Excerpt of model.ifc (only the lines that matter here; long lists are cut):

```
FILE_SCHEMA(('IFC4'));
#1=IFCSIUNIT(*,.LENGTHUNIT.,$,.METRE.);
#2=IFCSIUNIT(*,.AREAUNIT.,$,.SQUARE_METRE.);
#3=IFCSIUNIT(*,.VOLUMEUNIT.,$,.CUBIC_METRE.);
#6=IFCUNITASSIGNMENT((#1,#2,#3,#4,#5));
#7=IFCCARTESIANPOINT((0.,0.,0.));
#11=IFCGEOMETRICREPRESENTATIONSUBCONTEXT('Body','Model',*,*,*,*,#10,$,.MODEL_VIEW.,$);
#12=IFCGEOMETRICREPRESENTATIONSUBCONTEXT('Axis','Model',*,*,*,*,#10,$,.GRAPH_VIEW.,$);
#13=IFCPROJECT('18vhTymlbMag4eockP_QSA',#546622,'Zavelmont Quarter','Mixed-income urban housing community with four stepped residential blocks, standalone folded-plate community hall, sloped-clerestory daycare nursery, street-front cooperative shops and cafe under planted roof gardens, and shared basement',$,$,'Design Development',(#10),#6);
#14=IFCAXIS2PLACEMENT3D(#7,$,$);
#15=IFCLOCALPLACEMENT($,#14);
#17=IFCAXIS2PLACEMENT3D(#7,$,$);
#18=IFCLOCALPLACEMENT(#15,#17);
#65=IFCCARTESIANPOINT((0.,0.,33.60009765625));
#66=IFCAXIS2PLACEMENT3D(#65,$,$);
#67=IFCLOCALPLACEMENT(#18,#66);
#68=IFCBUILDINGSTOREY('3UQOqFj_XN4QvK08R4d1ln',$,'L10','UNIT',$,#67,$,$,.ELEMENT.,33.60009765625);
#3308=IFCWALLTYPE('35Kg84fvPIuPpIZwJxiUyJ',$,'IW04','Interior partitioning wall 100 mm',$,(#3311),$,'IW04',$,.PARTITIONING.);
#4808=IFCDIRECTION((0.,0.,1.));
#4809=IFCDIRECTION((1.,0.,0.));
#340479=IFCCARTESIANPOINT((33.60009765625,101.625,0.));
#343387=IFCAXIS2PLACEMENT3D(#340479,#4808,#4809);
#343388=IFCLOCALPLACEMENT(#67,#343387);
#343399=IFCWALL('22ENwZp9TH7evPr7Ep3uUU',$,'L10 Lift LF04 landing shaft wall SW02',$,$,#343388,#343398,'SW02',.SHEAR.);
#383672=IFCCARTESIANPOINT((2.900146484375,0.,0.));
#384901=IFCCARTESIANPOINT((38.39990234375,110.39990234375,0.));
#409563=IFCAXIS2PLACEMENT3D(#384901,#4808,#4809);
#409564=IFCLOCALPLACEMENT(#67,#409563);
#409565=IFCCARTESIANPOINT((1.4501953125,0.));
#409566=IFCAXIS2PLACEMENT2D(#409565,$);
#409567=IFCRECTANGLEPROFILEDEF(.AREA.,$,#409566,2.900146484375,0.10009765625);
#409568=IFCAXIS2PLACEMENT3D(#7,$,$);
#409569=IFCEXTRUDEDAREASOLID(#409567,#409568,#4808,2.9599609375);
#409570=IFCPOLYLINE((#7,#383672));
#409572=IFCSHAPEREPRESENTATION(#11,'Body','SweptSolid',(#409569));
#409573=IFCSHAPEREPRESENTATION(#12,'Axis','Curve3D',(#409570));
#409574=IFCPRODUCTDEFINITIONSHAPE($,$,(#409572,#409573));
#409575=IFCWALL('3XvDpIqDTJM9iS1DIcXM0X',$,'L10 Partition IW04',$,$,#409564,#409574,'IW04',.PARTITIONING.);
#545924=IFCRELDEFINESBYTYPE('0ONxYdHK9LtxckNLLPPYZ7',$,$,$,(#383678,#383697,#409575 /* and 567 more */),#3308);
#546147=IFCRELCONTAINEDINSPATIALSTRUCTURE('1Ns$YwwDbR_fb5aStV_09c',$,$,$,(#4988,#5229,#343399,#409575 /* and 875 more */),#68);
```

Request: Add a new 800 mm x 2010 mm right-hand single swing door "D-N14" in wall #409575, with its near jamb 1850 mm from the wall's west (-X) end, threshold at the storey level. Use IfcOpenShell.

```python
import numpy as np
import ifcopenshell
import ifcopenshell.api.feature
import ifcopenshell.api.geometry
import ifcopenshell.api.root
import ifcopenshell.api.spatial
import ifcopenshell.geom
import ifcopenshell.util.element
import ifcopenshell.util.placement
import ifcopenshell.util.representation
import ifcopenshell.util.shape
import ifcopenshell.util.unit

model = ifcopenshell.open("model.ifc")
unit_scale = ifcopenshell.util.unit.calculate_unit_scale(model)
settings = ifcopenshell.geom.settings()


def volume(element):
    """Net volume in cubic metres, openings subtracted."""
    shape = ifcopenshell.geom.create_shape(settings, element)
    return ifcopenshell.util.shape.get_volume(shape.geometry)


wall = model.by_id(409575)
storey = ifcopenshell.util.element.get_container(wall, ifc_class="IfcBuildingStorey")
context = ifcopenshell.util.representation.get_context(model, "Model", "Body", "MODEL_VIEW")
before = volume(wall)

width, height, from_end, sill = 0.8, 2.01, 1.85, 0.0  # metres

# The wall runs along its own X axis, and the end named is its -X end.
wall_shape = ifcopenshell.geom.create_shape(settings, wall)
x, y, z = ifcopenshell.util.shape.get_vertices(wall_shape.geometry).T
start = x.min() + from_end
face, thickness = float(y.min()), float(y.max() - y.min())
wall_matrix = ifcopenshell.util.placement.get_local_placement(wall.ObjectPlacement)
level = ifcopenshell.util.placement.get_local_placement(storey.ObjectPlacement)[2, 3]


def in_wall(x, y):
    """Placement at x, y metres in the wall's axes, at sill height."""
    matrix = wall_matrix.copy()
    matrix[:, 3] = wall_matrix @ np.array([x / unit_scale, y / unit_scale, 0.0, 1.0])
    matrix[2, 3] = level + sill / unit_scale
    return matrix


# Opening: a box that overshoots both wall faces by 50 mm.
opening = ifcopenshell.api.root.create_entity(model, ifc_class="IfcOpeningElement", predefined_type="OPENING")
box = ifcopenshell.api.geometry.add_wall_representation(
    model, context=context, length=width, height=height, thickness=thickness + 0.1
)
ifcopenshell.api.geometry.assign_representation(model, product=opening, representation=box)
ifcopenshell.api.geometry.edit_object_placement(model, product=opening, matrix=in_wall(start, face - 0.05), is_si=False)
ifcopenshell.api.feature.add_feature(model, feature=opening, element=wall)

door = ifcopenshell.api.root.create_entity(model, ifc_class="IfcDoor", name="D-N14", predefined_type="DOOR")
door.OverallWidth, door.OverallHeight = width / unit_scale, height / unit_scale
door.OperationType = "SINGLE_SWING_RIGHT"
body = ifcopenshell.api.geometry.add_door_representation(
    model,
    context=context,
    overall_width=door.OverallWidth,
    overall_height=door.OverallHeight,
    operation_type="SINGLE_SWING_RIGHT",
    lining_properties={"LiningDepth": thickness / unit_scale, "ThresholdDepth": thickness / unit_scale},
)
ifcopenshell.api.geometry.assign_representation(model, product=door, representation=body)
ifcopenshell.api.spatial.assign_container(model, products=[door], relating_structure=storey)
ifcopenshell.api.feature.add_filling(model, opening=opening, element=door)

# The lining spans the wall, so the door starts at the wall face.
ifcopenshell.api.geometry.edit_object_placement(model, product=door, matrix=in_wall(start, face), is_si=False)

after = volume(wall)

print(f"wall volume {before:.3f} -> {after:.3f} m3")

model.write("model_edited.ifc")
```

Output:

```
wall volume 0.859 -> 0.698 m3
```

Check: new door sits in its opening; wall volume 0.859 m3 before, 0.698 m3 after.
